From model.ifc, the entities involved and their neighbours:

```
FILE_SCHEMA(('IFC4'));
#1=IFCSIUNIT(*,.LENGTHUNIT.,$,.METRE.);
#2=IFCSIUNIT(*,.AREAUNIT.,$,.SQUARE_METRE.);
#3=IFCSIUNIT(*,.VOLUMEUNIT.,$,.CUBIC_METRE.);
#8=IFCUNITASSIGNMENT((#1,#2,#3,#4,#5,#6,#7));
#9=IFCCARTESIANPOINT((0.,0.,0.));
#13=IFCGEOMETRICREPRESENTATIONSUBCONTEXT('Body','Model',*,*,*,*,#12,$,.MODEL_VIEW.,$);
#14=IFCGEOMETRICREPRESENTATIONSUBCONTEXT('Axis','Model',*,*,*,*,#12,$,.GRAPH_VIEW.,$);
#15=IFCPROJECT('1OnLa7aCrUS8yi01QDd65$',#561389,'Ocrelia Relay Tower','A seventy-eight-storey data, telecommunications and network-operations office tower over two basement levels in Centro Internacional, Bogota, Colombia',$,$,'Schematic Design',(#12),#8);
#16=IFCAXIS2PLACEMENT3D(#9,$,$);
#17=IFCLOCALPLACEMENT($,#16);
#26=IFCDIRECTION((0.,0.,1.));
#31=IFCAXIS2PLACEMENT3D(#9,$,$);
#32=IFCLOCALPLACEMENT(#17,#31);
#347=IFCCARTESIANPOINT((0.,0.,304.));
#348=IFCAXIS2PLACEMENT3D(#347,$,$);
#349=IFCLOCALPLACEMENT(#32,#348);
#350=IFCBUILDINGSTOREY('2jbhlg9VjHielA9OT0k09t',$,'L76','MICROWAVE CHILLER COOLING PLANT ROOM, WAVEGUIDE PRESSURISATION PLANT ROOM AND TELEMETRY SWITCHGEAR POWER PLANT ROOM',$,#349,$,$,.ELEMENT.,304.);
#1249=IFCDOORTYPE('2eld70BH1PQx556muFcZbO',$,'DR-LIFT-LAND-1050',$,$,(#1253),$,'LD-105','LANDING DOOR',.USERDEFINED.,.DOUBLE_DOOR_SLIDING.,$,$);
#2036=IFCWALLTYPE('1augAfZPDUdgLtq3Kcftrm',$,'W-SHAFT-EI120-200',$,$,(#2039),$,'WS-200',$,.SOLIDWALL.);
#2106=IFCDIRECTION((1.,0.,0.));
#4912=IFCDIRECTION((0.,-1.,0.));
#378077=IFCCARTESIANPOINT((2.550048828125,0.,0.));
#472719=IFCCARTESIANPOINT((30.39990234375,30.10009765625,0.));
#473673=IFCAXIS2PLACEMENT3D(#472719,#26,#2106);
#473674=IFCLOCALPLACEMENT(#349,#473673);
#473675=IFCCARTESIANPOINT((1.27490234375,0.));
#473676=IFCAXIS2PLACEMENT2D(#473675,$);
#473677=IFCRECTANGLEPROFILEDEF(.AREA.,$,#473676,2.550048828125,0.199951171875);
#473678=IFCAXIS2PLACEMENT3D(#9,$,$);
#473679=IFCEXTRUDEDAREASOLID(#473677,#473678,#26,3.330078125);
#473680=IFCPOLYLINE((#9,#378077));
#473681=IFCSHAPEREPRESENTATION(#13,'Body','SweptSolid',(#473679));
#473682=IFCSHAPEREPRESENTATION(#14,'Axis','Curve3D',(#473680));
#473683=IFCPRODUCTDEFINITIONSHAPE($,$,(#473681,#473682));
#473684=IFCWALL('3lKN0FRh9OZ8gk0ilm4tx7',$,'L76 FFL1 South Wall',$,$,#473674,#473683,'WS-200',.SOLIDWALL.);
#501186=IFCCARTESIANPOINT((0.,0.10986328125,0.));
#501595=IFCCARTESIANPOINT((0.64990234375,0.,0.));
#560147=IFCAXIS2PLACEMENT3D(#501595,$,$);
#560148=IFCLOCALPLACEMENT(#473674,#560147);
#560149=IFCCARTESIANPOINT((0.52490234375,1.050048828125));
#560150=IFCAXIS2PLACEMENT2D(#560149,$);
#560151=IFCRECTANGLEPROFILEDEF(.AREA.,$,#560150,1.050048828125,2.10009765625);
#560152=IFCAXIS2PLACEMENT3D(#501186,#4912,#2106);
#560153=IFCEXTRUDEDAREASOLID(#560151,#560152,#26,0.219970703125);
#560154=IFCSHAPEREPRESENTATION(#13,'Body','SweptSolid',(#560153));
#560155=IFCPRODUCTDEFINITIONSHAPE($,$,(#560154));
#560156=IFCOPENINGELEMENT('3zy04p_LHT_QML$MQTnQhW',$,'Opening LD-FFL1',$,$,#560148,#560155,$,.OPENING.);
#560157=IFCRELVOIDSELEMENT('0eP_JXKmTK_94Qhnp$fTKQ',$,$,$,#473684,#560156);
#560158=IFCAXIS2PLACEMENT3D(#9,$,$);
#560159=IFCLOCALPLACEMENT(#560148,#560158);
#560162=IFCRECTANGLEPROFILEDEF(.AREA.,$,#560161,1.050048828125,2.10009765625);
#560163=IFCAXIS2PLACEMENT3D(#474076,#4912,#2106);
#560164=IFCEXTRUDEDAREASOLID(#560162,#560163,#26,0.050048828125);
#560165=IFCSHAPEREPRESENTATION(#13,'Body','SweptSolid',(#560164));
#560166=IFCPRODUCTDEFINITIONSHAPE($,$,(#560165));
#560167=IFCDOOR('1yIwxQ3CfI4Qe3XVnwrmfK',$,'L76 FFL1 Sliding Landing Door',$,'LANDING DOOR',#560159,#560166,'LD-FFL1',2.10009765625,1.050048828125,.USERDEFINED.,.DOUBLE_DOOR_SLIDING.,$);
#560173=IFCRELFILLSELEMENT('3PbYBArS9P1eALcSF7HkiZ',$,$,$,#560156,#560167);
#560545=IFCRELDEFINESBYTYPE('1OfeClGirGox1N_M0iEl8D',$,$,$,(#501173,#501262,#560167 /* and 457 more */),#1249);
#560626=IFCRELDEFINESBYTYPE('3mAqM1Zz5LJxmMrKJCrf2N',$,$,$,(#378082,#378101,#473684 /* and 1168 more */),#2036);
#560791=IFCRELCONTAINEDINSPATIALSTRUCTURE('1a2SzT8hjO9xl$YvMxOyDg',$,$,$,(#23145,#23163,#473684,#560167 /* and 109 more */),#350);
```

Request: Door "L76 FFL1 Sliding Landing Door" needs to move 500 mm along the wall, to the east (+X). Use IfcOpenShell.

```python
import ifcopenshell
import ifcopenshell.api.geometry
import ifcopenshell.util.placement
import ifcopenshell.util.unit

model = ifcopenshell.open("model.ifc")
unit_scale = ifcopenshell.util.unit.calculate_unit_scale(model)

door = model.by_guid("1yIwxQ3CfI4Qe3XVnwrmfK")
opening = door.FillsVoids[0].RelatingOpeningElement
wall = opening.VoidsElements[0].RelatingBuildingElement

wall_matrix = ifcopenshell.util.placement.get_local_placement(wall.ObjectPlacement)
shift = wall_matrix[:3, 0] * 0.5 / unit_scale
before = ifcopenshell.util.placement.get_local_placement(door.ObjectPlacement)[:3, 3].copy()

# The door is placed relative to its opening, so it follows when the opening moves.
matrix = ifcopenshell.util.placement.get_local_placement(opening.ObjectPlacement)
matrix[:3, 3] += shift
ifcopenshell.api.geometry.edit_object_placement(
    model, product=opening, matrix=matrix, is_si=False, should_transform_children=True
)

after = ifcopenshell.util.placement.get_local_placement(door.ObjectPlacement)[:3, 3]
print("door moved by", (after - before).round(3) + 0.0)

model.write("model_v2.ifc")
```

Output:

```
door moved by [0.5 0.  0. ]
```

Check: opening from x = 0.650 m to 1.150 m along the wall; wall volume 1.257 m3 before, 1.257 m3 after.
